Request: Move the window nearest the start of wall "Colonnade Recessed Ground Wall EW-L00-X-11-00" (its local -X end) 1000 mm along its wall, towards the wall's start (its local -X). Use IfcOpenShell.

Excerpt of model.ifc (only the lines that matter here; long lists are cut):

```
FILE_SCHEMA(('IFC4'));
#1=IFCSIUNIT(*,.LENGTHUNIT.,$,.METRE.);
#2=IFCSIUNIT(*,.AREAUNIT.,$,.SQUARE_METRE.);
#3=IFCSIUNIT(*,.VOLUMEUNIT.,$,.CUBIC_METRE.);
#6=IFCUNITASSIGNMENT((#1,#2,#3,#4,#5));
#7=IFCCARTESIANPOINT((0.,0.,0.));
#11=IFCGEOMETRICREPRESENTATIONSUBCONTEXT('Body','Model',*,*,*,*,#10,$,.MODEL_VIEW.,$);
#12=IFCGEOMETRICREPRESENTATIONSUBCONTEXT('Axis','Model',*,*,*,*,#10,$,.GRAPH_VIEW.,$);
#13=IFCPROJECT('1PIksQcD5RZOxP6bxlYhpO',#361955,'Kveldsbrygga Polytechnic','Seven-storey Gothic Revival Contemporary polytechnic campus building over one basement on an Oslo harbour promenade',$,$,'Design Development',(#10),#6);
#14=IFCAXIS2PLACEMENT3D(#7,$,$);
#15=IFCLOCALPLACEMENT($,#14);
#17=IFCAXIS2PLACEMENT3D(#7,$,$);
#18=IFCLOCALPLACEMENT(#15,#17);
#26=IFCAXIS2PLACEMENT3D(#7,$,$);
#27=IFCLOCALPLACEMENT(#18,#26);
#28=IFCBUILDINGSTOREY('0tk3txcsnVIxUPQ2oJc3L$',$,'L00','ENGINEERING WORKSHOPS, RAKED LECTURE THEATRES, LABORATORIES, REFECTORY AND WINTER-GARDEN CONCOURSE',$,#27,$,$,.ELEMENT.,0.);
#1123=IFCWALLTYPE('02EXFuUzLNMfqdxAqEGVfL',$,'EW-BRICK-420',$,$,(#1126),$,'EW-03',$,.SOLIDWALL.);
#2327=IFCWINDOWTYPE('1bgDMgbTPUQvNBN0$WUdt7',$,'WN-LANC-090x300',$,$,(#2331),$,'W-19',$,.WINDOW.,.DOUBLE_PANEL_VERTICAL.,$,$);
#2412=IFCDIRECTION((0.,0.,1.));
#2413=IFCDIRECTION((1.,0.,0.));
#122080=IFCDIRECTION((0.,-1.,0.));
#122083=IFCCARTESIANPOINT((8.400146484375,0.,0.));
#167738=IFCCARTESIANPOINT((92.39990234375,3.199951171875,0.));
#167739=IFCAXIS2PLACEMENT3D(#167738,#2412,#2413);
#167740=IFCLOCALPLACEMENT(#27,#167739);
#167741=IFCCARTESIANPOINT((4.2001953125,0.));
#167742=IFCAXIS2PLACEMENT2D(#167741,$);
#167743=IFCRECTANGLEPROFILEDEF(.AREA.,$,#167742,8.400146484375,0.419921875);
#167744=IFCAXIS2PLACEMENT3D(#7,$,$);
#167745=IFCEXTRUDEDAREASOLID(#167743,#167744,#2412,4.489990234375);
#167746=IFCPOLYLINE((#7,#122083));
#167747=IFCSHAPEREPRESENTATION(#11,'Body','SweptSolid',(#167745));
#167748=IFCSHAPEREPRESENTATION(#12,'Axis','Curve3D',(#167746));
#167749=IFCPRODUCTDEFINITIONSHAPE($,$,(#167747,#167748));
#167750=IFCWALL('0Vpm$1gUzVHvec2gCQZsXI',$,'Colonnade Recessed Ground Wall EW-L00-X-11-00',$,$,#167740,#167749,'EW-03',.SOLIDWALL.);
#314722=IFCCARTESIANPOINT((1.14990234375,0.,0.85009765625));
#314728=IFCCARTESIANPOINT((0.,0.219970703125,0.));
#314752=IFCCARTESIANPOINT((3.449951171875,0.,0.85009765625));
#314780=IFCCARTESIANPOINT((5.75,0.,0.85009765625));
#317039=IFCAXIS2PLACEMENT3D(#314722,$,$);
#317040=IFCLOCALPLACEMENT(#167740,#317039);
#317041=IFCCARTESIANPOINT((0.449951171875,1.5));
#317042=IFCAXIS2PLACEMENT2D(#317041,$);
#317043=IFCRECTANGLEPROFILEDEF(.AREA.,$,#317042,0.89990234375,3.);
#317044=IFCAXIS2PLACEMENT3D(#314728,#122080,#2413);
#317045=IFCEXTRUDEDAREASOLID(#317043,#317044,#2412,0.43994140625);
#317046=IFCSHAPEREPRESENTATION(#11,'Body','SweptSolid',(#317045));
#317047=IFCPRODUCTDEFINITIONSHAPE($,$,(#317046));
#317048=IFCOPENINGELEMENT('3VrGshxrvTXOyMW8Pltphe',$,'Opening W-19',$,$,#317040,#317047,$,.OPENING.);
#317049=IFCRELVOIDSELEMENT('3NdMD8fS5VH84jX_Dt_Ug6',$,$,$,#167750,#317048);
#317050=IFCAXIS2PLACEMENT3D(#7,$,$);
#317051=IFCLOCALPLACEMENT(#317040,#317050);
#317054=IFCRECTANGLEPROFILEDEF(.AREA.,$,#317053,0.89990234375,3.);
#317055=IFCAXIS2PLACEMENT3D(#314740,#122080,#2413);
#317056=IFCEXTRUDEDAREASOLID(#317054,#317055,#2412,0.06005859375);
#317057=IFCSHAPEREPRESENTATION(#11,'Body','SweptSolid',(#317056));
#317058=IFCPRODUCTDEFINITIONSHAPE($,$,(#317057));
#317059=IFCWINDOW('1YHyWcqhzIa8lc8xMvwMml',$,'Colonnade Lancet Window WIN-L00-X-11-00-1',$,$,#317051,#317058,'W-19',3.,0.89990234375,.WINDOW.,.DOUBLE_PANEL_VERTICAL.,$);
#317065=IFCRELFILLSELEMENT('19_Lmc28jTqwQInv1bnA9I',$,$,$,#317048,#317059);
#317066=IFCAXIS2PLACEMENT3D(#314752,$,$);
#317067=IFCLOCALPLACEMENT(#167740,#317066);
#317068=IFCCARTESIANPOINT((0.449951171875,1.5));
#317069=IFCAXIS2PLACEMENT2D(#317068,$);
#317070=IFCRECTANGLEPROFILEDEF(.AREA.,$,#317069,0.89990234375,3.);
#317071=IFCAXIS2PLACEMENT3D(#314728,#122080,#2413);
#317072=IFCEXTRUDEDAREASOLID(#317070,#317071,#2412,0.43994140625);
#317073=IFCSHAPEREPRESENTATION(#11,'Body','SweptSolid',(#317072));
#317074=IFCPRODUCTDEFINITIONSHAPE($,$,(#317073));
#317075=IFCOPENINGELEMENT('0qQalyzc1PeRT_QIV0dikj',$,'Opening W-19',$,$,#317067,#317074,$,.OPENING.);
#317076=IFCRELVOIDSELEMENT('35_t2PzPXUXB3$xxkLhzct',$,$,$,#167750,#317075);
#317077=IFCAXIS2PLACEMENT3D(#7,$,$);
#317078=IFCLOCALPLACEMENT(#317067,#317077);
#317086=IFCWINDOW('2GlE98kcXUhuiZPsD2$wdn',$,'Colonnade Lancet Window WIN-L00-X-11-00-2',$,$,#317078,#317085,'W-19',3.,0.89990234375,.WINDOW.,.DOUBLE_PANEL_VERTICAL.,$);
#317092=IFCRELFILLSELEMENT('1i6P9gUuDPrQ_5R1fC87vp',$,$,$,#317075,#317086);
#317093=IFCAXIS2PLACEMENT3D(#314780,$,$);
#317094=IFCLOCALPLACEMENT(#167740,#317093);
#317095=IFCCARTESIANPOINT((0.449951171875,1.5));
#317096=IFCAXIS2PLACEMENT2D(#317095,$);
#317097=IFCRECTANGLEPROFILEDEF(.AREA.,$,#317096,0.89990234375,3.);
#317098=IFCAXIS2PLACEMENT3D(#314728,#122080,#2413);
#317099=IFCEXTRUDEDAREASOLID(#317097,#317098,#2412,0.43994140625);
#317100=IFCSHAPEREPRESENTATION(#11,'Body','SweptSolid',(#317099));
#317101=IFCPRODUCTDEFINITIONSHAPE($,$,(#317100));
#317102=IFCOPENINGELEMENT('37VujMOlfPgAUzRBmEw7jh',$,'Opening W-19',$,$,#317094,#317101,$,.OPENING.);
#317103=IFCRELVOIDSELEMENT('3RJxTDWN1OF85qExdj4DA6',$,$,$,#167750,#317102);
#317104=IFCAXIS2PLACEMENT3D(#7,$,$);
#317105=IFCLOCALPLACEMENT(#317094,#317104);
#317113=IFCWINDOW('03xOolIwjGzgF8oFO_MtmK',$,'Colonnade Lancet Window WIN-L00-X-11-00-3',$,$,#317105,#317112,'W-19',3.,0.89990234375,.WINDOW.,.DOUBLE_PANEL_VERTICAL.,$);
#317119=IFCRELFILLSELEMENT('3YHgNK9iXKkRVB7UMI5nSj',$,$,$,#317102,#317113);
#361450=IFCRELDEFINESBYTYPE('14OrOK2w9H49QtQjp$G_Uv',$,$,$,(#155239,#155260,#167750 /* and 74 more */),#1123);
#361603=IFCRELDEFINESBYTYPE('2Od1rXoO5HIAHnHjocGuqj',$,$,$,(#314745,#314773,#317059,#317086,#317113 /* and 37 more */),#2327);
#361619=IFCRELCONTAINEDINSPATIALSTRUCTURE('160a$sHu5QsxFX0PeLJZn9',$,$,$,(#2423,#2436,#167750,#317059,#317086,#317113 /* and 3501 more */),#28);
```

```python
import ifcopenshell
import ifcopenshell.api.geometry
import ifcopenshell.util.placement

model = ifcopenshell.open("model.ifc")

window = model.by_guid("1YHyWcqhzIa8lc8xMvwMml")
opening = window.FillsVoids[0].RelatingOpeningElement
wall = opening.VoidsElements[0].RelatingBuildingElement

wall_matrix = ifcopenshell.util.placement.get_local_placement(wall.ObjectPlacement)
shift = wall_matrix[:3, 0] * -1.0
before = ifcopenshell.util.placement.get_local_placement(window.ObjectPlacement)[:3, 3].copy()

# The window is placed relative to its opening, so it follows when the opening moves.
matrix = ifcopenshell.util.placement.get_local_placement(opening.ObjectPlacement)
matrix[:3, 3] += shift
ifcopenshell.api.geometry.edit_object_placement(
    model, product=opening, matrix=matrix, is_si=False, should_transform_children=True
)

after = ifcopenshell.util.placement.get_local_placement(window.ObjectPlacement)[:3, 3]
print("window moved by", (after - before).round(3) + 0.0)

model.write("model_rev.ifc")
```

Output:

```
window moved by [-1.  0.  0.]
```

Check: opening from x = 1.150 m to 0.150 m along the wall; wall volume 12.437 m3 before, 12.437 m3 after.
